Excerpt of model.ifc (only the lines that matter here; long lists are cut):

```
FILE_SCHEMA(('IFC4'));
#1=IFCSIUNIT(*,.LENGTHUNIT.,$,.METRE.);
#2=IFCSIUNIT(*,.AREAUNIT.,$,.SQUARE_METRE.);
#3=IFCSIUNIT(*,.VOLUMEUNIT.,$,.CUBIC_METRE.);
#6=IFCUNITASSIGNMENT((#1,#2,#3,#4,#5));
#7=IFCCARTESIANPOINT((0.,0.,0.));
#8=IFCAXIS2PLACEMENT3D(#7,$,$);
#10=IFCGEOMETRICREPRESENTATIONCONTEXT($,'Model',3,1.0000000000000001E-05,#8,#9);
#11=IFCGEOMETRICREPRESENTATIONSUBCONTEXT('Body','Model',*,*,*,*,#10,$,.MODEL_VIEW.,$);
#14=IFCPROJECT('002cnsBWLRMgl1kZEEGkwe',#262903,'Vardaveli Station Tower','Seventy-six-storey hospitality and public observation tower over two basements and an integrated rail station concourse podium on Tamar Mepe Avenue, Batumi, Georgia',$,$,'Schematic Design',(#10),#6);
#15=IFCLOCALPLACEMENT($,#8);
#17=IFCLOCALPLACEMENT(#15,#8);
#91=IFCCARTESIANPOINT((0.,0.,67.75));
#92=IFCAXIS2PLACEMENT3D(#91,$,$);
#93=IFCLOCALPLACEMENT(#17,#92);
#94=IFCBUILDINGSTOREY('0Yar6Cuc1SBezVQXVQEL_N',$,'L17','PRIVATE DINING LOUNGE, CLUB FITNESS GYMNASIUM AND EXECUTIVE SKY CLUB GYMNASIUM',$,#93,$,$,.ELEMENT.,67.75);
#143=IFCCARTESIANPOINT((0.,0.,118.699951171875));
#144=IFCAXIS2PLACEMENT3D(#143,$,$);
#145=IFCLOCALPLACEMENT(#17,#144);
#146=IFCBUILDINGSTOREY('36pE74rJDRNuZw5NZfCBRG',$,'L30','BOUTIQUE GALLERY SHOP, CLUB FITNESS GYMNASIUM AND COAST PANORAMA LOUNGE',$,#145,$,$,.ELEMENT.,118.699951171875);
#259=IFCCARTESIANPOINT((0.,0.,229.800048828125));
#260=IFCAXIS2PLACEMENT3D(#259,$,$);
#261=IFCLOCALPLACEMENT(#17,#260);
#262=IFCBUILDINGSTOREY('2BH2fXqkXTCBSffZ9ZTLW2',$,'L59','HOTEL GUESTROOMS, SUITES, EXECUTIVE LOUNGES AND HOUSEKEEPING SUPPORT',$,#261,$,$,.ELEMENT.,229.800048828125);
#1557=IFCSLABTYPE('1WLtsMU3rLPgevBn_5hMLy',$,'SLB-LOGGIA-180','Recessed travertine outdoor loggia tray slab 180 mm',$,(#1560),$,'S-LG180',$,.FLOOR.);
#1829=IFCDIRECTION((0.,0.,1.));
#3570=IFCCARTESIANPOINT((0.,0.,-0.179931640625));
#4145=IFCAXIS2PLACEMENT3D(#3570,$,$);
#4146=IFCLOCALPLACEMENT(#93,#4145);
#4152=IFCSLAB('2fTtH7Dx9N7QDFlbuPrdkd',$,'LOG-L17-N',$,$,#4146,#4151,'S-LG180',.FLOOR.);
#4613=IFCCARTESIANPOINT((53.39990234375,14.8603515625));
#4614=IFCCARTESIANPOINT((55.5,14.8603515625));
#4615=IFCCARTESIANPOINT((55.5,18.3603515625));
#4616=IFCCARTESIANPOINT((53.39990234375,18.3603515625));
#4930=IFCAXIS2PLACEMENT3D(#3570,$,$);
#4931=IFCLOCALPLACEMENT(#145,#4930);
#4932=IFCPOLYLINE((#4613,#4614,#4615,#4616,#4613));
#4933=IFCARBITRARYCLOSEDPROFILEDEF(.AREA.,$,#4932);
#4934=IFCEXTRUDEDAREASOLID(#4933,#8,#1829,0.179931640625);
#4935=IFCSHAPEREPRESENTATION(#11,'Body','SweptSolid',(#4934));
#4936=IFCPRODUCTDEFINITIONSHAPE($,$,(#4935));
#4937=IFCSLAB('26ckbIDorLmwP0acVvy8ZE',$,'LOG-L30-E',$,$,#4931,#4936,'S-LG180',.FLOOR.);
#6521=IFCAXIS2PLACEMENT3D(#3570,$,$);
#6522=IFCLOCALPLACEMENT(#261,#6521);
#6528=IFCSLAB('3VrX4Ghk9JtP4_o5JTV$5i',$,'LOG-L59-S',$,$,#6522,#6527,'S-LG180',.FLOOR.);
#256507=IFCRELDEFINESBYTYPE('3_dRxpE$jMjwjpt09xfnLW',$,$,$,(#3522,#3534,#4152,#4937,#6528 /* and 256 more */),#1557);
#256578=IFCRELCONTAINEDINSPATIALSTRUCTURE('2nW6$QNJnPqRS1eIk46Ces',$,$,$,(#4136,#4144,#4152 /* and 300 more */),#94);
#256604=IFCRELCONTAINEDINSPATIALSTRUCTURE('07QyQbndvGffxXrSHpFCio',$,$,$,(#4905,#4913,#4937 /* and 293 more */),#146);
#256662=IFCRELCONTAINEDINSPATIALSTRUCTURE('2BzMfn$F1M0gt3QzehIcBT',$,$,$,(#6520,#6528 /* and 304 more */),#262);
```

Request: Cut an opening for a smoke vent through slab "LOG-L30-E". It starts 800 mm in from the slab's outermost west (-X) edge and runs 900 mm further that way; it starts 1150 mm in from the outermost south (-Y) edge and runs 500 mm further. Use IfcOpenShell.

```python
import numpy as np
import ifcopenshell
import ifcopenshell.api.feature
import ifcopenshell.api.geometry
import ifcopenshell.api.root
import ifcopenshell.geom
import ifcopenshell.util.placement
import ifcopenshell.util.representation
import ifcopenshell.util.shape
import ifcopenshell.util.unit

model = ifcopenshell.open("model.ifc")
unit_scale = ifcopenshell.util.unit.calculate_unit_scale(model)
settings = ifcopenshell.geom.settings()


def volume(element):
    """Net volume in cubic metres, openings subtracted."""
    shape = ifcopenshell.geom.create_shape(settings, element)
    return ifcopenshell.util.shape.get_volume(shape.geometry)


slab = model.by_guid("26ckbIDorLmwP0acVvy8ZE")
before = volume(slab)

# Extent in the slab's own axes, in metres. The edges named are its -X and -Y sides.
slab_shape = ifcopenshell.geom.create_shape(settings, slab)
vertices = ifcopenshell.util.shape.get_vertices(slab_shape.geometry)
x_min, y_min, bottom = vertices.min(axis=0)
top = vertices[:, 2].max()

opening = ifcopenshell.api.root.create_entity(model, ifc_class="IfcOpeningElement", name="Smoke vent opening", predefined_type="OPENING")
context = ifcopenshell.util.representation.get_context(model, "Model", "Body", "MODEL_VIEW")
width, depth = 0.9, 0.5
outline = [(0.0, 0.0), (width, 0.0), (width, depth), (0.0, depth), (0.0, 0.0)]
# Overshoot both faces by 50 mm so the cut is clean.
shape = ifcopenshell.api.geometry.add_slab_representation(
    model, context=context, depth=top - bottom + 0.1, polyline=outline
)
ifcopenshell.api.geometry.assign_representation(model, product=opening, representation=shape)

matrix = ifcopenshell.util.placement.get_local_placement(slab.ObjectPlacement)
matrix[:, 3] = matrix @ np.append(np.array([x_min + 0.8, y_min + 1.15, bottom - 0.05]) / unit_scale, 1.0)
ifcopenshell.api.geometry.edit_object_placement(model, product=opening, matrix=matrix, is_si=False)
ifcopenshell.api.feature.add_feature(model, feature=opening, element=slab)

after = volume(slab)

print(f"slab volume {before:.3f} -> {after:.3f} m3")

model.write("model-out.ifc")
```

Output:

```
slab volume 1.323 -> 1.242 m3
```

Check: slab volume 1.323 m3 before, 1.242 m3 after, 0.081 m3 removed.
